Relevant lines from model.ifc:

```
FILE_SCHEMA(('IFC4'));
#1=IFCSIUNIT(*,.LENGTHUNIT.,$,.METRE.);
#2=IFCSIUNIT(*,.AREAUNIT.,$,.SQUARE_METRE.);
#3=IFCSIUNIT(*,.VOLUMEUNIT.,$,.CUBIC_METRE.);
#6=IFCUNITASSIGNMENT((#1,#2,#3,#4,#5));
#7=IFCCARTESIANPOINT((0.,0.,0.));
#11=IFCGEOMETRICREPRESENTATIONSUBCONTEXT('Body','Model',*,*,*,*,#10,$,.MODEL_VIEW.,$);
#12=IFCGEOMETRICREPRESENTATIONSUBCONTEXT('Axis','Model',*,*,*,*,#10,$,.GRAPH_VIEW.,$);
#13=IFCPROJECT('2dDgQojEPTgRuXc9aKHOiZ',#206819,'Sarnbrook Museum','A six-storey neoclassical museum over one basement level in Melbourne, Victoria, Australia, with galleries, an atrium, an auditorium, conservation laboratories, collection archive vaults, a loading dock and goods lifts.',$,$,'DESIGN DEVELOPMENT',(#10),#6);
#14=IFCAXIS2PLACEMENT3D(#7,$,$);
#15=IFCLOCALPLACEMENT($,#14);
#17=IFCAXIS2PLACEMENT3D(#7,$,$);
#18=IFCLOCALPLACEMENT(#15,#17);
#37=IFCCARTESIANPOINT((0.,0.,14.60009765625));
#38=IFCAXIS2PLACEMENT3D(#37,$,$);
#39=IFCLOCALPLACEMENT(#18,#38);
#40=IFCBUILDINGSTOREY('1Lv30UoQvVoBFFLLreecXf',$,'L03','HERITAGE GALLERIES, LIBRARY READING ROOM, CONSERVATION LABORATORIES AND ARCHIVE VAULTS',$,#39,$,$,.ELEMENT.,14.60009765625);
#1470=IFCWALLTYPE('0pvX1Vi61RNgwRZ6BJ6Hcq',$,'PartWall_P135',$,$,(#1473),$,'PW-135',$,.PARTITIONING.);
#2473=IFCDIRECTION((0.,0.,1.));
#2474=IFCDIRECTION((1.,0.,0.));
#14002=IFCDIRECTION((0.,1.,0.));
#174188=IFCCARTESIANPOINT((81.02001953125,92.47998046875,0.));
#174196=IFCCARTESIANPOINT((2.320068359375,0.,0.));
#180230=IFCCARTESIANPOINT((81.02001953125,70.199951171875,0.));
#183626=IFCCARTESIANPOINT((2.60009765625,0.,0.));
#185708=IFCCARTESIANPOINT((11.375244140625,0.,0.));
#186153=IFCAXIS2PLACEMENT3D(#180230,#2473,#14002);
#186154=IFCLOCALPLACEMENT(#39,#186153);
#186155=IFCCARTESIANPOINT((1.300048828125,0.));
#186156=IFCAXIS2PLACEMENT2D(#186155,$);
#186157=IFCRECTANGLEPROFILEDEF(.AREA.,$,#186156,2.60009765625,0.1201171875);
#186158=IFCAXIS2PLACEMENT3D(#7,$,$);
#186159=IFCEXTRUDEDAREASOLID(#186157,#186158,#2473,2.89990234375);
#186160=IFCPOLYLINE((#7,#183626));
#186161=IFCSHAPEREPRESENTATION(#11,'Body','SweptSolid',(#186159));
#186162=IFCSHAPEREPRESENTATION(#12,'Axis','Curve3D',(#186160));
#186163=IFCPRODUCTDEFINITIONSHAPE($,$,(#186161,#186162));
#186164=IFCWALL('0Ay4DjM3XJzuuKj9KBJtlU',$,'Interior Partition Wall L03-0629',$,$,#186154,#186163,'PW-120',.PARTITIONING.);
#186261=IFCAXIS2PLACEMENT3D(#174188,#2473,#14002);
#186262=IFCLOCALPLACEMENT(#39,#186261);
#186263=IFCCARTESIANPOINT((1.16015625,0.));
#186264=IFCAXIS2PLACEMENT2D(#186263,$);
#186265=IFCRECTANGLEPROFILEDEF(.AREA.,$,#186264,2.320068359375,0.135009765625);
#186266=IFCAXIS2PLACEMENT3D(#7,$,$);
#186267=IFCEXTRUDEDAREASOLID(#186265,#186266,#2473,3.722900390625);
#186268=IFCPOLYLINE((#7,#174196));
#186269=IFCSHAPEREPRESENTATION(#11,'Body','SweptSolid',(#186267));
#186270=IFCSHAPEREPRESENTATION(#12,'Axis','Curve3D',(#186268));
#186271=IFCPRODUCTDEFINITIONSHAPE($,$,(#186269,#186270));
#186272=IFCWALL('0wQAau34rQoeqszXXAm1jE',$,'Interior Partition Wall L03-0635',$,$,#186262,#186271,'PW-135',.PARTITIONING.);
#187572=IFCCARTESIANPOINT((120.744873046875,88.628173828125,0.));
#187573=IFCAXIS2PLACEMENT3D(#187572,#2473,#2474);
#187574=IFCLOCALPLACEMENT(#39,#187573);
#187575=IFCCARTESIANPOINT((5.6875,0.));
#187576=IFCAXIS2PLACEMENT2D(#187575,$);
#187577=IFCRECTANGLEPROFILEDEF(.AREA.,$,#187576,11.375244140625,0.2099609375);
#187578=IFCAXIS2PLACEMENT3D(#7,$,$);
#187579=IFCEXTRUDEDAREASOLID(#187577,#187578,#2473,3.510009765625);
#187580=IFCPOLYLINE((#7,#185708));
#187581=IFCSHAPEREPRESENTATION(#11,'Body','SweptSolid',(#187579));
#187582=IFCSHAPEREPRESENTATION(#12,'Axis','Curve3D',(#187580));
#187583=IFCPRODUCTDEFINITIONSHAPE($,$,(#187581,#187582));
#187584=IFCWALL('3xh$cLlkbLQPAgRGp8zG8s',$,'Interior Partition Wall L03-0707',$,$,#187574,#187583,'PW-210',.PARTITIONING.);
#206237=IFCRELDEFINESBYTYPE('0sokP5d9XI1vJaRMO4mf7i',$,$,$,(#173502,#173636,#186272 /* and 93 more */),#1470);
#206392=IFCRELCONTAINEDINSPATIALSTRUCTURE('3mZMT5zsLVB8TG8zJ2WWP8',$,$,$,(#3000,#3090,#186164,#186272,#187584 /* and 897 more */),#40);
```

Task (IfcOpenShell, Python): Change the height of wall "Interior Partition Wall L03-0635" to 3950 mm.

```python
import ifcopenshell
import ifcopenshell.geom
import ifcopenshell.util.representation
import ifcopenshell.util.shape
import ifcopenshell.util.unit

model = ifcopenshell.open("model.ifc")
unit_scale = ifcopenshell.util.unit.calculate_unit_scale(model)
settings = ifcopenshell.geom.settings()


def volume(element):
    """Net volume in cubic metres, openings subtracted."""
    shape = ifcopenshell.geom.create_shape(settings, element)
    return ifcopenshell.util.shape.get_volume(shape.geometry)


wall = model.by_guid("0wQAau34rQoeqszXXAm1jE")
before = volume(wall)

body = ifcopenshell.util.representation.get_representation(wall, "Model", "Body")
solid = body.Items[0]
old_height = solid.Depth
solid.Depth = 3.95 / unit_scale
after = volume(wall)

print(f"height {old_height:g} -> {solid.Depth:g}, volume {before:.3f} -> {after:.3f} m3")

model.write("model-out.ifc")
```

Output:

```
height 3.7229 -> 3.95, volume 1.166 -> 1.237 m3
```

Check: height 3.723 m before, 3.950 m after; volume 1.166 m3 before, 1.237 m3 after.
